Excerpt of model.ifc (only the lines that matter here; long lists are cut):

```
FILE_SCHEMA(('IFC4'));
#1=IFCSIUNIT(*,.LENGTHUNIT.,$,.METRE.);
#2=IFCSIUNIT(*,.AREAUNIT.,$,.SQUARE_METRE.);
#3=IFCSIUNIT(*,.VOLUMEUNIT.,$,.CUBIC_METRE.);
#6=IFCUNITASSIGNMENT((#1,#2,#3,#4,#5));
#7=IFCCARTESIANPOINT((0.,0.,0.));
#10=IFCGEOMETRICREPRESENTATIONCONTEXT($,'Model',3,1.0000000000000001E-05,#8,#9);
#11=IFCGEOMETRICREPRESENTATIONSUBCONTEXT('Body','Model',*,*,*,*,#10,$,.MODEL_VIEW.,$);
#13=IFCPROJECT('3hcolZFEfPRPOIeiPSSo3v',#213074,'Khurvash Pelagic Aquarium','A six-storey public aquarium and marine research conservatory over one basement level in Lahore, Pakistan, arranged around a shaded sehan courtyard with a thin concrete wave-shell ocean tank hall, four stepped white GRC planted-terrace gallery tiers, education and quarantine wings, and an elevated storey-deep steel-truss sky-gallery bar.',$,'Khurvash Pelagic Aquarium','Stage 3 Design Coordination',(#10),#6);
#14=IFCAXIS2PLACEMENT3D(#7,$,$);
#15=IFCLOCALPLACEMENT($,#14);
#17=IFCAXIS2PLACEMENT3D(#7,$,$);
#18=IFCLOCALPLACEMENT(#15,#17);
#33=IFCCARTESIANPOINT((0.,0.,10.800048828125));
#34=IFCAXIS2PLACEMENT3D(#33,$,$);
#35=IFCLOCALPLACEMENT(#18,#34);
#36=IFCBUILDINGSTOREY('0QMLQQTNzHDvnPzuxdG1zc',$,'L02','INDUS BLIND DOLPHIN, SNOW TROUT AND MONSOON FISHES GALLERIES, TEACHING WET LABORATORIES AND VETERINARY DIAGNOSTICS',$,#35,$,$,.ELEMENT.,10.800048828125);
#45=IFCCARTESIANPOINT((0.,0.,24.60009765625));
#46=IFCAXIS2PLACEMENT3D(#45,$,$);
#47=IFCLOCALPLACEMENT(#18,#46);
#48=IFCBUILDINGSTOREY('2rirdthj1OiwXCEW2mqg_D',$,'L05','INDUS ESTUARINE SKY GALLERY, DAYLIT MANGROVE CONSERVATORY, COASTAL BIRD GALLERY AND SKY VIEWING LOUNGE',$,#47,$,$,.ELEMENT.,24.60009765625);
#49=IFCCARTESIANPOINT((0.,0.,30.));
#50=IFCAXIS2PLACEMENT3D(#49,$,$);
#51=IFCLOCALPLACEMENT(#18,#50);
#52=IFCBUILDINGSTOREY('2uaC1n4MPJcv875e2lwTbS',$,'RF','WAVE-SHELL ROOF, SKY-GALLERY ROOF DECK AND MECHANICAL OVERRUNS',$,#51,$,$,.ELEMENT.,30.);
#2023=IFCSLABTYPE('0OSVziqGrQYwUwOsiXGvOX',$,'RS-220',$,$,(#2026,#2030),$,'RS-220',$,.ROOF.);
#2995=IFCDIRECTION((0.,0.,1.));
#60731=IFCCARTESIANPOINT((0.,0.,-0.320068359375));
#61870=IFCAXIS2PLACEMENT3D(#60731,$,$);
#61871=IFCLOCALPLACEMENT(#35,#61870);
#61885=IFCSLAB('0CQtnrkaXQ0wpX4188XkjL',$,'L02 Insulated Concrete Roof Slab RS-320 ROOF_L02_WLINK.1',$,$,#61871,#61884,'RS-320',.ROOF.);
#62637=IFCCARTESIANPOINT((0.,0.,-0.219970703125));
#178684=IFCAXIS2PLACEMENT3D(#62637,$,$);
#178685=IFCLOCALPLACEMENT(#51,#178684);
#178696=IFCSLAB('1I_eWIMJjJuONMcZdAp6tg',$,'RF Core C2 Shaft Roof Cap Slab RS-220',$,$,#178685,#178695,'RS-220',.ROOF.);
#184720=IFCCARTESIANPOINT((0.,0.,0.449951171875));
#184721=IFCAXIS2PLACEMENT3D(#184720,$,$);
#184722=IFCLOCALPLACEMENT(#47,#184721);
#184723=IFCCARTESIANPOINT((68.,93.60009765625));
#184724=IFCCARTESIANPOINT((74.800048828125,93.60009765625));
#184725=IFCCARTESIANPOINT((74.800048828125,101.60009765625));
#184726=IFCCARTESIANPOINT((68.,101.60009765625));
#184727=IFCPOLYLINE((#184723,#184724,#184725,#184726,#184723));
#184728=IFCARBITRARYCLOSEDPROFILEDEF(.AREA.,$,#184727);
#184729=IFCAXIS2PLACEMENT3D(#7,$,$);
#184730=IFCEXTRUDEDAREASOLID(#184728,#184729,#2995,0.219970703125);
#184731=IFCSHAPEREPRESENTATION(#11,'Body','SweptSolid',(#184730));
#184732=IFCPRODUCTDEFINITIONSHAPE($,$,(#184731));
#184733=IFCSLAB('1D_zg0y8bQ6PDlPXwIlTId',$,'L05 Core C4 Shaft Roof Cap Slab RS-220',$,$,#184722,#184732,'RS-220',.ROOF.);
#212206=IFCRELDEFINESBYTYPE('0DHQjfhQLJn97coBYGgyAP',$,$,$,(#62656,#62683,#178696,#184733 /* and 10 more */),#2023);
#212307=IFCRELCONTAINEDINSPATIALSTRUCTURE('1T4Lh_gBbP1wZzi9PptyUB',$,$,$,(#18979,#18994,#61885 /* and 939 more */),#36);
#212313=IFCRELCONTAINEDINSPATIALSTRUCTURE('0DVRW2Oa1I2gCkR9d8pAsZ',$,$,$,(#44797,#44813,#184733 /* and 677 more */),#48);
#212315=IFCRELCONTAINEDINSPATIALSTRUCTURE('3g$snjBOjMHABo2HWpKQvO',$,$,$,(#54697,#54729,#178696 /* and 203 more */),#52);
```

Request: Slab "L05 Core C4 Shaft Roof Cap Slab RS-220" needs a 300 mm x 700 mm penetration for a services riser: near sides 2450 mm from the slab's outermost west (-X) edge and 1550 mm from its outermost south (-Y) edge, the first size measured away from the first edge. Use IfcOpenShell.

```python
import numpy as np
import ifcopenshell
import ifcopenshell.api.feature
import ifcopenshell.api.geometry
import ifcopenshell.api.root
import ifcopenshell.geom
import ifcopenshell.util.placement
import ifcopenshell.util.representation
import ifcopenshell.util.shape
import ifcopenshell.util.unit

model = ifcopenshell.open("model.ifc")
unit_scale = ifcopenshell.util.unit.calculate_unit_scale(model)
settings = ifcopenshell.geom.settings()


def volume(element):
    """Net volume in cubic metres, openings subtracted."""
    shape = ifcopenshell.geom.create_shape(settings, element)
    return ifcopenshell.util.shape.get_volume(shape.geometry)


slab = model.by_guid("1D_zg0y8bQ6PDlPXwIlTId")
before = volume(slab)

# Extent in the slab's own axes, in metres. The edges named are its -X and -Y sides.
slab_shape = ifcopenshell.geom.create_shape(settings, slab)
vertices = ifcopenshell.util.shape.get_vertices(slab_shape.geometry)
x_min, y_min, bottom = vertices.min(axis=0)
top = vertices[:, 2].max()

opening = ifcopenshell.api.root.create_entity(model, ifc_class="IfcOpeningElement", name="Services riser opening", predefined_type="OPENING")
context = ifcopenshell.util.representation.get_context(model, "Model", "Body", "MODEL_VIEW")
width, depth = 0.3, 0.7
outline = [(0.0, 0.0), (width, 0.0), (width, depth), (0.0, depth), (0.0, 0.0)]
# Overshoot both faces by 50 mm so the cut is clean.
shape = ifcopenshell.api.geometry.add_slab_representation(
    model, context=context, depth=top - bottom + 0.1, polyline=outline
)
ifcopenshell.api.geometry.assign_representation(model, product=opening, representation=shape)

matrix = ifcopenshell.util.placement.get_local_placement(slab.ObjectPlacement)
matrix[:, 3] = matrix @ np.append(np.array([x_min + 2.45, y_min + 1.55, bottom - 0.05]) / unit_scale, 1.0)
ifcopenshell.api.geometry.edit_object_placement(model, product=opening, matrix=matrix, is_si=False)
ifcopenshell.api.feature.add_feature(model, feature=opening, element=slab)

after = volume(slab)

print(f"slab volume {before:.3f} -> {after:.3f} m3")

model.write("model_v2.ifc")
```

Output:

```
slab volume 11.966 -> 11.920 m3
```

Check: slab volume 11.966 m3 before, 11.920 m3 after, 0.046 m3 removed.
